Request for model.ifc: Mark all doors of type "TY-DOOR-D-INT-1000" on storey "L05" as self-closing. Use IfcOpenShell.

First a look at what the model holds.

```python
import ifcopenshell
import ifcopenshell.util.element

model = ifcopenshell.open("model.ifc")
print(model.schema)
storey = next(s for s in model.by_type("IfcBuildingStorey") if s.Name == "L05")
doors = [e for e in ifcopenshell.util.element.get_decomposition(storey) if e.is_a("IfcDoor")]
seen = {}
for e in doors:
    element_type = ifcopenshell.util.element.get_type(e)
    key = (element_type.Name if element_type != e and element_type else None, ifcopenshell.util.element.get_pset(e, "Pset_DoorCommon", "SelfClosing"))
    seen[key] = seen.get(key, 0) + 1
for (name, value), count in sorted(seen.items(), key=str):
    print(count, "x", name, "|", value)
```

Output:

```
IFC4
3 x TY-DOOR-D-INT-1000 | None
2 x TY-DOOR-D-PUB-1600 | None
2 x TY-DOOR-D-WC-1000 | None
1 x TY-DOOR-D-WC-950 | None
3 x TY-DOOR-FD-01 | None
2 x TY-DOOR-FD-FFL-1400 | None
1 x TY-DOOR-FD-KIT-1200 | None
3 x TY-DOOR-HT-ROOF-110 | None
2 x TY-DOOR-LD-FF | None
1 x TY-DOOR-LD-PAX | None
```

```python
import ifcopenshell
import ifcopenshell.api.pset
import ifcopenshell.util.element

model = ifcopenshell.open("model.ifc")

storey = next(s for s in model.by_type("IfcBuildingStorey") if s.Name == "L05")
doors = [e for e in ifcopenshell.util.element.get_decomposition(storey) if e.is_a("IfcDoor")]

count = 0
for e in doors:
    element_type = ifcopenshell.util.element.get_type(e)
    if element_type in (None, e) or element_type.Name != "TY-DOOR-D-INT-1000":
        continue
    # add_pset returns the element's existing set when there is one.
    pset = ifcopenshell.api.pset.add_pset(model, product=e, name="Pset_DoorCommon")
    ifcopenshell.api.pset.edit_pset(model, pset=pset, properties={"SelfClosing": True})
    count += 1

print(count, "doors updated")

model.write("model_v2.ifc")
```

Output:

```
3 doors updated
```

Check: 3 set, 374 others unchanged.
